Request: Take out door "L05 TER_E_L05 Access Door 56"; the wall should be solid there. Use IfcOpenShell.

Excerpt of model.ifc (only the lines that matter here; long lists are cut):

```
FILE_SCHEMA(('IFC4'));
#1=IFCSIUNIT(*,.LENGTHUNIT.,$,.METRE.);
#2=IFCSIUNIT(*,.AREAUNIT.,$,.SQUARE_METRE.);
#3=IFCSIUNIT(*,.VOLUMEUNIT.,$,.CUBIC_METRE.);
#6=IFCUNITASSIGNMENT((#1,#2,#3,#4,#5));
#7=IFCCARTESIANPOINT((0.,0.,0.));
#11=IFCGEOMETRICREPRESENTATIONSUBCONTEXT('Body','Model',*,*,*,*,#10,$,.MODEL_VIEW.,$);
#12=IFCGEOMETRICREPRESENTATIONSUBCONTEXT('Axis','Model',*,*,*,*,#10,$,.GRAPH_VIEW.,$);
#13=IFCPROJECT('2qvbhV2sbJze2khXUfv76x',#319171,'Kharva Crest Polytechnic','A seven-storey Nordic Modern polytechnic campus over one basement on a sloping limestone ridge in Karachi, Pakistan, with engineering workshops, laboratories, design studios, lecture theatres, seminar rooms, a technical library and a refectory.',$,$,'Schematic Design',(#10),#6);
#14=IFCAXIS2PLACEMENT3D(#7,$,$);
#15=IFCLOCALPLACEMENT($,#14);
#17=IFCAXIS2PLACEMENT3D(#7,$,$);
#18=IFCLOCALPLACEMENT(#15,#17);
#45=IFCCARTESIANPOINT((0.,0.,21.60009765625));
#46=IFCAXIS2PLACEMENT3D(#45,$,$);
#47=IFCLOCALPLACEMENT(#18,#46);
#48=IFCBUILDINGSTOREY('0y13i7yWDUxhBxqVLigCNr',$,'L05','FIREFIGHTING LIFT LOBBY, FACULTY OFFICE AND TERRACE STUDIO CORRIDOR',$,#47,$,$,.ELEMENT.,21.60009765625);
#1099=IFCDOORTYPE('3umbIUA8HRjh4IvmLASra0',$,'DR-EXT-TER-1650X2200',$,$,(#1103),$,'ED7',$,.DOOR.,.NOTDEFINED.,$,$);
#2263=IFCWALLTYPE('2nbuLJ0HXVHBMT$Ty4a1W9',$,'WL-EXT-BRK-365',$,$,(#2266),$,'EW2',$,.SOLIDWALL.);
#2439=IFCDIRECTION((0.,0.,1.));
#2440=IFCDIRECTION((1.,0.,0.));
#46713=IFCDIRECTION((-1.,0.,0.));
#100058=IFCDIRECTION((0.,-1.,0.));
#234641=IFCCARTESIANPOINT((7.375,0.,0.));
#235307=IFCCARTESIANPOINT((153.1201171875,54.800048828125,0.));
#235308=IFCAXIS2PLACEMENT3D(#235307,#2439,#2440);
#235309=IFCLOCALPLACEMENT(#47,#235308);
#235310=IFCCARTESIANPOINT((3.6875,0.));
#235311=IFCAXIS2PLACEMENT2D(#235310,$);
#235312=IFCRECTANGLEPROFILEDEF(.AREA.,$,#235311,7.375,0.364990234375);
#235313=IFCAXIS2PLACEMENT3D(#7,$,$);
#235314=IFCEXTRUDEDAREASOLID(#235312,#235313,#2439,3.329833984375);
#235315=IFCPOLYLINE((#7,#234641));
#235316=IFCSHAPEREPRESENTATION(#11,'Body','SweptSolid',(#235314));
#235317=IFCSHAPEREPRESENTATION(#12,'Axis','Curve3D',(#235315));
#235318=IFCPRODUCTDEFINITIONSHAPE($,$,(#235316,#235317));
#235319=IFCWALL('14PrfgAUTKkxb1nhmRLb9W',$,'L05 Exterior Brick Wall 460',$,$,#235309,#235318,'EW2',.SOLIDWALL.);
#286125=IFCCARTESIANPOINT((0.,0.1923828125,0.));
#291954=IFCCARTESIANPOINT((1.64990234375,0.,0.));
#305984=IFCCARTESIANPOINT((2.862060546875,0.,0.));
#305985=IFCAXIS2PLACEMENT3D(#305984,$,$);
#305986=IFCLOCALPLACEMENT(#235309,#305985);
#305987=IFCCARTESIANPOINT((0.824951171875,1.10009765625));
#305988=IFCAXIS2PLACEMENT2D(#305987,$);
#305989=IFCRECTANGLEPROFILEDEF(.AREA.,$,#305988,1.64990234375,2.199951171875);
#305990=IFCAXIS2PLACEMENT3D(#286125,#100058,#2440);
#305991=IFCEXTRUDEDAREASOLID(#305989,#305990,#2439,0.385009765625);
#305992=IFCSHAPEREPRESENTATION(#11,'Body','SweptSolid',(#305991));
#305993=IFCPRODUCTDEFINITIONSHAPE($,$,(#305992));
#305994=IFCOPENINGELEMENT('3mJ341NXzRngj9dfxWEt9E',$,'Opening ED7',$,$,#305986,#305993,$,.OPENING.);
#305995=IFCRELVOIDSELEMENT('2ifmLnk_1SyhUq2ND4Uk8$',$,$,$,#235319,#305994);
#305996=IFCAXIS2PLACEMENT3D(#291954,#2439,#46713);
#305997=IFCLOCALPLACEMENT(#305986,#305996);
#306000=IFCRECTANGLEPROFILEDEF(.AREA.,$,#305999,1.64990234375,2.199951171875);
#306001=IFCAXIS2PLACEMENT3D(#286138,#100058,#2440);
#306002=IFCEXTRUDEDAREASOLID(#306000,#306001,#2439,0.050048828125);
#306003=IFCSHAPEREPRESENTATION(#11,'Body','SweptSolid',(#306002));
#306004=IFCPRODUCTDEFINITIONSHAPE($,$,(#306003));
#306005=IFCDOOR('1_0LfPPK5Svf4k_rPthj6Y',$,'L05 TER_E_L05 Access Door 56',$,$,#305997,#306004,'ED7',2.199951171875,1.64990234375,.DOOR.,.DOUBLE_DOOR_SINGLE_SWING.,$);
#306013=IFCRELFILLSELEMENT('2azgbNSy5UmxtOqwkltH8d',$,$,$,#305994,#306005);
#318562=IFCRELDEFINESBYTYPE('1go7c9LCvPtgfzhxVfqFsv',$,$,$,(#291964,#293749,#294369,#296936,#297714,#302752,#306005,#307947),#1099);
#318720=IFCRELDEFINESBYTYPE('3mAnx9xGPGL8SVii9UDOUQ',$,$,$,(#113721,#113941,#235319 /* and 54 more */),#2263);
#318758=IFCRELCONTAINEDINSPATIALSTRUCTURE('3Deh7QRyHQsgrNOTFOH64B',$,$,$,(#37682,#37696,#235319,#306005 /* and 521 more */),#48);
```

```python
import ifcopenshell
import ifcopenshell.api.feature
import ifcopenshell.api.root
import ifcopenshell.geom
import ifcopenshell.util.shape

model = ifcopenshell.open("model.ifc")
settings = ifcopenshell.geom.settings()


def volume(element):
    """Net volume in cubic metres, openings subtracted."""
    shape = ifcopenshell.geom.create_shape(settings, element)
    return ifcopenshell.util.shape.get_volume(shape.geometry)


door = model.by_id(306005)
opening = door.FillsVoids[0].RelatingOpeningElement
wall = opening.VoidsElements[0].RelatingBuildingElement
before = volume(wall)

ifcopenshell.api.root.remove_product(model, product=door)
ifcopenshell.api.feature.remove_feature(model, feature=opening)

after = volume(wall)

print(f"wall volume {before:.3f} -> {after:.3f} m3")

model.write("model_edited.ifc")
```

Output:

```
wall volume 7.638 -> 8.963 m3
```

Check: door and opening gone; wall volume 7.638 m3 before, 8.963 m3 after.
